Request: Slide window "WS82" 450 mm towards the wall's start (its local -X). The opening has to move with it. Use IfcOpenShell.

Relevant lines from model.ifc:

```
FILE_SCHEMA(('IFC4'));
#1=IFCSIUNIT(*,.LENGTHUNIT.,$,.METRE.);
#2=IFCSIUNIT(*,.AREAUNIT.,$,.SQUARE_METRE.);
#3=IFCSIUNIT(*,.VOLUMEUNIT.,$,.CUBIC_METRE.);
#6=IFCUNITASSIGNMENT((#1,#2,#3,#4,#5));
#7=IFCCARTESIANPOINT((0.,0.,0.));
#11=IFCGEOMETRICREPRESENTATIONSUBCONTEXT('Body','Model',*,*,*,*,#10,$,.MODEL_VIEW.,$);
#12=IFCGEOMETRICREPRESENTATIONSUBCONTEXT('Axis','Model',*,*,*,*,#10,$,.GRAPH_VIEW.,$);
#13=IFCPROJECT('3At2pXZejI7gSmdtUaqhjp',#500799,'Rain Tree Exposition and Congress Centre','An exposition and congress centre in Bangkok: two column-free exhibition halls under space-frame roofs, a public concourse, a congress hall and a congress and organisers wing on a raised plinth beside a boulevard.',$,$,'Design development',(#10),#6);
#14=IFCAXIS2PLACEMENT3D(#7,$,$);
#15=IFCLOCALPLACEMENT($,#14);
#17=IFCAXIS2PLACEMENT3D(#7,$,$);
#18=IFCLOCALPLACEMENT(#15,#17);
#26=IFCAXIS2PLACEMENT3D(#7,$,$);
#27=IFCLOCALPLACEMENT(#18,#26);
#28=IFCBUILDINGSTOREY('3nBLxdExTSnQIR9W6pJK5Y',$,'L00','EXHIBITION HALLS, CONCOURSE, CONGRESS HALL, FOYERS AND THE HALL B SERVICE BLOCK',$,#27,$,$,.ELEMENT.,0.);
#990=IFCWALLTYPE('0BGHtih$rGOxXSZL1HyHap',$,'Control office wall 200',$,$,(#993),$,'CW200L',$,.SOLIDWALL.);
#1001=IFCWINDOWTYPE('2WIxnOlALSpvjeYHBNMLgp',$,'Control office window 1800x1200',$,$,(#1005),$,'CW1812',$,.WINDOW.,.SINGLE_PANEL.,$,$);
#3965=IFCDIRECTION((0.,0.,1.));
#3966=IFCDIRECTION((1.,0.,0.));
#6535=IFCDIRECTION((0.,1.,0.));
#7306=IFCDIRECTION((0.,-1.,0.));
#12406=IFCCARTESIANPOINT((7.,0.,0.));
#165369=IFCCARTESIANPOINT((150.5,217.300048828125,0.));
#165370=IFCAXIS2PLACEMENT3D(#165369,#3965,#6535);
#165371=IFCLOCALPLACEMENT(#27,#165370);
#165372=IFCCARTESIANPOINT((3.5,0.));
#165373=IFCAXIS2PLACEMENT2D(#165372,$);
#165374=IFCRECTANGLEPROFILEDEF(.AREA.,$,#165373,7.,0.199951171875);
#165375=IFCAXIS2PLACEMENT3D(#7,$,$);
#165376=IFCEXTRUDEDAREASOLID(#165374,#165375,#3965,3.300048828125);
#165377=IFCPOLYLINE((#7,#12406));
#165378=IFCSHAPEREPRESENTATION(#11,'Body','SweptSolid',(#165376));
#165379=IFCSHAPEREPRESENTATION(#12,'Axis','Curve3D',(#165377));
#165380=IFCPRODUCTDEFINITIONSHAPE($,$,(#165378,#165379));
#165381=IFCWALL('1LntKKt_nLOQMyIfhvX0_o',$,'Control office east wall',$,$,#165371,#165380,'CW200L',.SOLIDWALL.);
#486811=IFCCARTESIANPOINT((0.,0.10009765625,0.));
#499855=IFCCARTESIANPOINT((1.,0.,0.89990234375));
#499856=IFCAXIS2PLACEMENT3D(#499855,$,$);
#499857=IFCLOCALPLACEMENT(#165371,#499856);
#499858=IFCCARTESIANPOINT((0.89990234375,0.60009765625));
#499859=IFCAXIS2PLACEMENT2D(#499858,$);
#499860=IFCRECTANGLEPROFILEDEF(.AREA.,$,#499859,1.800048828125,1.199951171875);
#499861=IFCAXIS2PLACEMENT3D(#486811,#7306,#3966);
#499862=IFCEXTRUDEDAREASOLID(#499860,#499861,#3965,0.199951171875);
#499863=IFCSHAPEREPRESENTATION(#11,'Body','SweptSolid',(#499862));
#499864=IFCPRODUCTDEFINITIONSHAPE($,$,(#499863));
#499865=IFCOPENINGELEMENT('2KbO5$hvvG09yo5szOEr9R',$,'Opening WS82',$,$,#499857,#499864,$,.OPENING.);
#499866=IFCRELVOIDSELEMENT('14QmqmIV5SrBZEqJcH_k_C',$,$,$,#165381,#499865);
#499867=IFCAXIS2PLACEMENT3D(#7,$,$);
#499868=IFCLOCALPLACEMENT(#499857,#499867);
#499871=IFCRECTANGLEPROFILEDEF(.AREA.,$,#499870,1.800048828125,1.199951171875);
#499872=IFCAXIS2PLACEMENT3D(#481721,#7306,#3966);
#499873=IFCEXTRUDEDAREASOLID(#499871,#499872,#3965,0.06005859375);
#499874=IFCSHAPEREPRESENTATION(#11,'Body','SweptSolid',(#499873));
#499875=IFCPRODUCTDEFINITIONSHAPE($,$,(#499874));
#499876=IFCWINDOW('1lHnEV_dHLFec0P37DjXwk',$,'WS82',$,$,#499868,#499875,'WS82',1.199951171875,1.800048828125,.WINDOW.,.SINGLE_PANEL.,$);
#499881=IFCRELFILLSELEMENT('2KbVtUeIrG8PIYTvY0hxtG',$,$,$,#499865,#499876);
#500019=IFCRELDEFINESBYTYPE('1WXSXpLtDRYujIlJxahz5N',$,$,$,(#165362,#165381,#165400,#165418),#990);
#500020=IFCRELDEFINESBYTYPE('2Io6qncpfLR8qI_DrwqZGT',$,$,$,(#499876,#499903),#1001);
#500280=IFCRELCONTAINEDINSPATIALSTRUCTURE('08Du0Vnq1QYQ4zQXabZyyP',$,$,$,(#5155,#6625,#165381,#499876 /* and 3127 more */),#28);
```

```python
import ifcopenshell
import ifcopenshell.api.geometry
import ifcopenshell.util.placement
import ifcopenshell.util.unit

model = ifcopenshell.open("model.ifc")
unit_scale = ifcopenshell.util.unit.calculate_unit_scale(model)

window = model.by_id(499876)
opening = window.FillsVoids[0].RelatingOpeningElement
wall = opening.VoidsElements[0].RelatingBuildingElement

wall_matrix = ifcopenshell.util.placement.get_local_placement(wall.ObjectPlacement)
shift = wall_matrix[:3, 0] * -0.45 / unit_scale
before = ifcopenshell.util.placement.get_local_placement(window.ObjectPlacement)[:3, 3].copy()

# The window is placed relative to its opening, so it follows when the opening moves.
matrix = ifcopenshell.util.placement.get_local_placement(opening.ObjectPlacement)
matrix[:3, 3] += shift
ifcopenshell.api.geometry.edit_object_placement(
    model, product=opening, matrix=matrix, is_si=False, should_transform_children=True
)

after = ifcopenshell.util.placement.get_local_placement(window.ObjectPlacement)[:3, 3]
print("window moved by", (after - before).round(3) + 0.0)

model.write("model_v2.ifc")
```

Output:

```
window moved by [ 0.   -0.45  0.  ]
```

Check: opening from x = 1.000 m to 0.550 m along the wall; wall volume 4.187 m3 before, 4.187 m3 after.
